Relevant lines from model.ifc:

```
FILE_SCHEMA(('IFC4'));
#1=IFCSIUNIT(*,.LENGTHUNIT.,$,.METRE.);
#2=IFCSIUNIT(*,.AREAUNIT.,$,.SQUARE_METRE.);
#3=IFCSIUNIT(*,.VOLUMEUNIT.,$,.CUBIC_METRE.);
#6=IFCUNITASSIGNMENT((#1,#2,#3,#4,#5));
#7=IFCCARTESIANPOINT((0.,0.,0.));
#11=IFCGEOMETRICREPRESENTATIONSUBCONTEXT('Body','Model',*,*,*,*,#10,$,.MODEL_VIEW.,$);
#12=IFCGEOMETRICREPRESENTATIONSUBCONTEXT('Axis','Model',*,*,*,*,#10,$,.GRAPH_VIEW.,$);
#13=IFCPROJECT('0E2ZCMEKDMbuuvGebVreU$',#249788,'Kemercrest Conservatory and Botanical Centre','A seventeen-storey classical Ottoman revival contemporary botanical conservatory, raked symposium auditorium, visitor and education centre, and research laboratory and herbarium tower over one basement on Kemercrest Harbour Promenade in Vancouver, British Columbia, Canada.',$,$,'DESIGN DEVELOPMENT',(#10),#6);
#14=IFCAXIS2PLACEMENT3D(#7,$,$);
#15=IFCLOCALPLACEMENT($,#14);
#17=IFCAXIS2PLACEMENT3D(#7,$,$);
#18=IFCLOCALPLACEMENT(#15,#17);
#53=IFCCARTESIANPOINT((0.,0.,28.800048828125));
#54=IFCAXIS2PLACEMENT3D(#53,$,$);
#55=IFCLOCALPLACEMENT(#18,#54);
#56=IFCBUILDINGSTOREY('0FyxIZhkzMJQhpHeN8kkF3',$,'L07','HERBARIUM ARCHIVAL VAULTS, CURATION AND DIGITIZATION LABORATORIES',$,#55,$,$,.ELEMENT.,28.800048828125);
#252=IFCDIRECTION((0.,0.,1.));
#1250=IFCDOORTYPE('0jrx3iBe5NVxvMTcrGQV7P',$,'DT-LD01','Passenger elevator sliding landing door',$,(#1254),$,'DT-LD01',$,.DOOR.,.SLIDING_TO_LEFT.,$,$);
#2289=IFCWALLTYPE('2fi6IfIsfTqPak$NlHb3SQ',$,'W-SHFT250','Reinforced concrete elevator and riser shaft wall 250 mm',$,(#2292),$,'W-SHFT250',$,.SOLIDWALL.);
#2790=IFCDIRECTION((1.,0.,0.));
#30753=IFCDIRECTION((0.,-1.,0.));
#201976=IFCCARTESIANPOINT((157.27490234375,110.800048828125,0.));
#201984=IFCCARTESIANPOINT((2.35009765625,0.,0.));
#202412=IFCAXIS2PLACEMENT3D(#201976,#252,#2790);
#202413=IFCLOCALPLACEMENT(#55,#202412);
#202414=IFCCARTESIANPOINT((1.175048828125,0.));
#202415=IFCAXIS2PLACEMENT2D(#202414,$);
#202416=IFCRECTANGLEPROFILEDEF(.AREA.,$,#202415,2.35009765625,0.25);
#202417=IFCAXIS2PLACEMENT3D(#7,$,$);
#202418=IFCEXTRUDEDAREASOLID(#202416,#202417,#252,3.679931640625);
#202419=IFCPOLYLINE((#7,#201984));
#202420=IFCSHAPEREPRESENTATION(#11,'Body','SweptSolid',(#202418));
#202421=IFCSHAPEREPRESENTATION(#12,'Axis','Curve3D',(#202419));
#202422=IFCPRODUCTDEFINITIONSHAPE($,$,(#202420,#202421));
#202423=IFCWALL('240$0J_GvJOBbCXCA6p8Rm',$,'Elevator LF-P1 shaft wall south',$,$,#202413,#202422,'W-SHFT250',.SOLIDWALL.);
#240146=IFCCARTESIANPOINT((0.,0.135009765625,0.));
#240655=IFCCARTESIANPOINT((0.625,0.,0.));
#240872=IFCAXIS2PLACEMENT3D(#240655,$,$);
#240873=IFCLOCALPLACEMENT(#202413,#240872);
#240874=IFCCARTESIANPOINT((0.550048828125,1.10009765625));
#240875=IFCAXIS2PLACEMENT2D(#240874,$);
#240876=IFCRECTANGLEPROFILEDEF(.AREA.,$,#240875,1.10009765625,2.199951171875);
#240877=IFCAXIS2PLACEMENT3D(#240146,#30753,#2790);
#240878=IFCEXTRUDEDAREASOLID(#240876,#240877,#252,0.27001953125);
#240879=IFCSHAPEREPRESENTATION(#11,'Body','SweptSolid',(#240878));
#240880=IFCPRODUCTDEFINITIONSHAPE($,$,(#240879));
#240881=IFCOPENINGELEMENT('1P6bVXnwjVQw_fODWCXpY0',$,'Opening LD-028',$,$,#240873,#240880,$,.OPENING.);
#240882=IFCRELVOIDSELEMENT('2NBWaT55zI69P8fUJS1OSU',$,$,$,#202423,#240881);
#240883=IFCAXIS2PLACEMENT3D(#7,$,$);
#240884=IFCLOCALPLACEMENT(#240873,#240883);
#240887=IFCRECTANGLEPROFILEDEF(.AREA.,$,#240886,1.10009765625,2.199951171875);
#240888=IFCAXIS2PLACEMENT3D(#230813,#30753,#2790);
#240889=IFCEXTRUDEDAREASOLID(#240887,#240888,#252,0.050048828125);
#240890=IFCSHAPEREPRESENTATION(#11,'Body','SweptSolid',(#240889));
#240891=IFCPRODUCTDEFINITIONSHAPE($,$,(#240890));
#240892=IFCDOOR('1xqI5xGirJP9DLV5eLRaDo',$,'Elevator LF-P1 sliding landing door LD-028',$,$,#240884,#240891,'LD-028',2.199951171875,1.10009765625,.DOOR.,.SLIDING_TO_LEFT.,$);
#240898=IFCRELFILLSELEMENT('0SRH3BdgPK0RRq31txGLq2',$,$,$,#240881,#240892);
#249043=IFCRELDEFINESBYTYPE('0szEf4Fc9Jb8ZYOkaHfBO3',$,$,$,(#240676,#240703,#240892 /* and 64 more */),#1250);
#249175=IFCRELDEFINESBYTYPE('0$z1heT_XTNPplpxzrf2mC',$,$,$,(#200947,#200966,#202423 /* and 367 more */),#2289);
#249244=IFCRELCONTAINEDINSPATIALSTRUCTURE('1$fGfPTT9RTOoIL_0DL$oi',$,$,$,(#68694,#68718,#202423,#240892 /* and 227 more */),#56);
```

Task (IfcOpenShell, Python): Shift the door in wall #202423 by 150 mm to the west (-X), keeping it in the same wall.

```python
import ifcopenshell
import ifcopenshell.api.geometry
import ifcopenshell.util.placement

model = ifcopenshell.open("model.ifc")

door = model.by_id(240892)
opening = door.FillsVoids[0].RelatingOpeningElement
wall = opening.VoidsElements[0].RelatingBuildingElement

wall_matrix = ifcopenshell.util.placement.get_local_placement(wall.ObjectPlacement)
shift = wall_matrix[:3, 0] * -0.15
before = ifcopenshell.util.placement.get_local_placement(door.ObjectPlacement)[:3, 3].copy()

# The door is placed relative to its opening, so it follows when the opening moves.
matrix = ifcopenshell.util.placement.get_local_placement(opening.ObjectPlacement)
matrix[:3, 3] += shift
ifcopenshell.api.geometry.edit_object_placement(
    model, product=opening, matrix=matrix, is_si=False, should_transform_children=True
)

after = ifcopenshell.util.placement.get_local_placement(door.ObjectPlacement)[:3, 3]
print("door moved by", (after - before).round(3) + 0.0)

model.write("model-out.ifc")
```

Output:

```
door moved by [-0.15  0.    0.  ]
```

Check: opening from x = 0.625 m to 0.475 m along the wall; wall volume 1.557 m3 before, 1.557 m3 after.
